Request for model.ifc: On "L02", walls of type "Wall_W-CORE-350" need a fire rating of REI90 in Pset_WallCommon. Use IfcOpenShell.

First a look at what the model holds.

```python
import ifcopenshell
import ifcopenshell.util.element

model = ifcopenshell.open("model.ifc")
print(model.schema)
storey = next(s for s in model.by_type("IfcBuildingStorey") if s.Name == "L02")
walls = [e for e in ifcopenshell.util.element.get_decomposition(storey) if e.is_a("IfcWall")]
seen = {}
for e in walls:
    element_type = ifcopenshell.util.element.get_type(e)
    key = (element_type.Name if element_type != e and element_type else None, ifcopenshell.util.element.get_pset(e, "Pset_WallCommon", "FireRating"))
    seen[key] = seen.get(key, 0) + 1
for (name, value), count in sorted(seen.items(), key=str):
    print(count, "x", name, "|", value)
```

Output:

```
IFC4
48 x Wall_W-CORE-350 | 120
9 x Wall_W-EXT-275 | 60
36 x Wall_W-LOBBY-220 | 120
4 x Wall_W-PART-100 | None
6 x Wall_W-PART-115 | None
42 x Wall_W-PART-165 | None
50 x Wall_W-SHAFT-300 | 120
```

```python
import ifcopenshell
import ifcopenshell.api.pset
import ifcopenshell.util.element

model = ifcopenshell.open("model.ifc")

storey = next(s for s in model.by_type("IfcBuildingStorey") if s.Name == "L02")
walls = [e for e in ifcopenshell.util.element.get_decomposition(storey) if e.is_a("IfcWall")]

count = 0
for e in walls:
    element_type = ifcopenshell.util.element.get_type(e)
    if element_type in (None, e) or element_type.Name != "Wall_W-CORE-350":
        continue
    # add_pset returns the element's existing set when there is one.
    pset = ifcopenshell.api.pset.add_pset(model, product=e, name="Pset_WallCommon")
    ifcopenshell.api.pset.edit_pset(model, pset=pset, properties={"FireRating": "REI90"})
    count += 1

print(count, "walls updated")

model.write("model_edited.ifc")
```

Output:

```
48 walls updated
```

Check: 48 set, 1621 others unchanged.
